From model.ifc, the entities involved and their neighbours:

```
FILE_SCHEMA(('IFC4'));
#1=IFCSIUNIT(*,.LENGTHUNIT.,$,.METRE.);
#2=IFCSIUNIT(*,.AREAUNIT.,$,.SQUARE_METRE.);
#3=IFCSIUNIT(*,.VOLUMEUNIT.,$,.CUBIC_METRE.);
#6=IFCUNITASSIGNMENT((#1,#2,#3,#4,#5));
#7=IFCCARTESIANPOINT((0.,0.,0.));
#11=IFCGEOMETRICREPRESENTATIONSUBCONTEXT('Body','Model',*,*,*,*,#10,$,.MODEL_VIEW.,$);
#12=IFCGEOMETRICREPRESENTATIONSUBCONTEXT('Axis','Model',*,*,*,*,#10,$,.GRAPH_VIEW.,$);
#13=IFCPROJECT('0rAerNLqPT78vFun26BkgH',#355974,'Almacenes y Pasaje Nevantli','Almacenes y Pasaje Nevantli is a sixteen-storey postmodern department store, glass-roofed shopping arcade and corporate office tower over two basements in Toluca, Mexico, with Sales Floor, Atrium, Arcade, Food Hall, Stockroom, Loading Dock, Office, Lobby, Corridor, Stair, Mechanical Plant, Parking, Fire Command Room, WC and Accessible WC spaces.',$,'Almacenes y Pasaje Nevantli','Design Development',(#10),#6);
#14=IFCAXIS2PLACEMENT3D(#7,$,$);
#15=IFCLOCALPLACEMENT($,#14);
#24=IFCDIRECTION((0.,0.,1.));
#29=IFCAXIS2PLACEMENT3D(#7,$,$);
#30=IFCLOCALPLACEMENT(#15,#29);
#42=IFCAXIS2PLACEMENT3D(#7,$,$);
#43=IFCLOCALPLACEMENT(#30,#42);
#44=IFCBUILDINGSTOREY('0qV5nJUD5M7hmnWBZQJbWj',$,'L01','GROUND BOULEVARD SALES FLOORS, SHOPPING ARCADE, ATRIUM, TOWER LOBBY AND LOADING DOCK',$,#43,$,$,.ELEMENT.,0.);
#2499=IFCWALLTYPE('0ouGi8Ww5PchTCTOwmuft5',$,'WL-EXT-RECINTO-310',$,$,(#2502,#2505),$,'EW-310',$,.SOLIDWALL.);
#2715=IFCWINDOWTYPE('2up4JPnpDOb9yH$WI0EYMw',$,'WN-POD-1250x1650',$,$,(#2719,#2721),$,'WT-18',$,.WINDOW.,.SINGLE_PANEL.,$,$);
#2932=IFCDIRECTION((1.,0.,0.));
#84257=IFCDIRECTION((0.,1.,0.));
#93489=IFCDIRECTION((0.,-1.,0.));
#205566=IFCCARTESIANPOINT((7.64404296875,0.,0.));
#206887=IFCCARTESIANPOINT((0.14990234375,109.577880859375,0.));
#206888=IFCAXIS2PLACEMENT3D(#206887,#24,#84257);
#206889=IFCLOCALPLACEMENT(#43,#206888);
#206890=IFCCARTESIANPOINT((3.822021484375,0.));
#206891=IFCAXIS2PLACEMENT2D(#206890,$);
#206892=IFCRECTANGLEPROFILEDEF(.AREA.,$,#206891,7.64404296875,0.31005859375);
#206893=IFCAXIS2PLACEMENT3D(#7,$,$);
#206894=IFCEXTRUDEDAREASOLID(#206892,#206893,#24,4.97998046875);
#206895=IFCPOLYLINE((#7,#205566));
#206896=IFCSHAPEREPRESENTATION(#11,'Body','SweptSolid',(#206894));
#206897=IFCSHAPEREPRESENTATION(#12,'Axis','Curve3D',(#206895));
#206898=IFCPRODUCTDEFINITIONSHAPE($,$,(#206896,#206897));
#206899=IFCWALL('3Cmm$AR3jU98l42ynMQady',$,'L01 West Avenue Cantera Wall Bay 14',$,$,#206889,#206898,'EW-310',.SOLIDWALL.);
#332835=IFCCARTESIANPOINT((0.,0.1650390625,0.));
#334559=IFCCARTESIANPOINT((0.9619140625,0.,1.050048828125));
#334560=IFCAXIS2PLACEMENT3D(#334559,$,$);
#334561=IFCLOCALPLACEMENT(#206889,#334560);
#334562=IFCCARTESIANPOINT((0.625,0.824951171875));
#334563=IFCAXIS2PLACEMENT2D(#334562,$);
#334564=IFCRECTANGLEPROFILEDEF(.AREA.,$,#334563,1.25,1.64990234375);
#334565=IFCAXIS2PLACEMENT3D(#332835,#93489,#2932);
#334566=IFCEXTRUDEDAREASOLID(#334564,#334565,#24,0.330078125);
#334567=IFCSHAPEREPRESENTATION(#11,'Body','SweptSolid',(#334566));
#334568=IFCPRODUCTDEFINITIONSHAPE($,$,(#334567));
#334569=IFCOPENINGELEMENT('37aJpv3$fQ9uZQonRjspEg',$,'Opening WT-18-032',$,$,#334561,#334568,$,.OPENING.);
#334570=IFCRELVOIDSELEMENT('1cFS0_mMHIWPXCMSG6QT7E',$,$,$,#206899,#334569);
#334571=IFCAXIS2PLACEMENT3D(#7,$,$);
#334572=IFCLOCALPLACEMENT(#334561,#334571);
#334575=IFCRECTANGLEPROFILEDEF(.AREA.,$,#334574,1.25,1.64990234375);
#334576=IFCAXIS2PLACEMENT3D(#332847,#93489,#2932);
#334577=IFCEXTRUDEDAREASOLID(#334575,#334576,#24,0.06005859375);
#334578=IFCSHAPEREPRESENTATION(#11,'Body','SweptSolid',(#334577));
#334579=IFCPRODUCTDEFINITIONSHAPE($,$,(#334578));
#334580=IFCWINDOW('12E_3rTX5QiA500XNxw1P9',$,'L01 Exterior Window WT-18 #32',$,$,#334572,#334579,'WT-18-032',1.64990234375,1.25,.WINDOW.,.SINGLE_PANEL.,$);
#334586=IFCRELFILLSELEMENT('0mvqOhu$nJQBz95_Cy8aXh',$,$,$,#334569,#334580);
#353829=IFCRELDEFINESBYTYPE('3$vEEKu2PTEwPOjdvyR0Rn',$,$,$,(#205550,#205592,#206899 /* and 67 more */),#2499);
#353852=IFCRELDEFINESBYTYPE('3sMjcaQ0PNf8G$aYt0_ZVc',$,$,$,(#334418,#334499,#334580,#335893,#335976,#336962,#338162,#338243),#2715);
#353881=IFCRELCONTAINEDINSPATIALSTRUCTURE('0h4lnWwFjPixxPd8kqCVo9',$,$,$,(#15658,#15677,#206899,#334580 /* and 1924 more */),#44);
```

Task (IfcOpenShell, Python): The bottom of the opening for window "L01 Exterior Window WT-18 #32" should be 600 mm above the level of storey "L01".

```python
import numpy as np
import ifcopenshell
import ifcopenshell.api.geometry
import ifcopenshell.geom
import ifcopenshell.util.element
import ifcopenshell.util.placement
import ifcopenshell.util.shape
import ifcopenshell.util.unit

model = ifcopenshell.open("model.ifc")
unit_scale = ifcopenshell.util.unit.calculate_unit_scale(model)

window = model.by_guid("12E_3rTX5QiA500XNxw1P9")
opening = window.FillsVoids[0].RelatingOpeningElement
storey = ifcopenshell.util.element.get_container(window, ifc_class="IfcBuildingStorey")
level = ifcopenshell.util.placement.get_local_placement(storey.ObjectPlacement)[2, 3]

# The opening's origin need not be at the sill, so measure its lowest point.
shape = ifcopenshell.geom.create_shape(ifcopenshell.geom.settings(), opening)
bottom = ifcopenshell.util.shape.get_shape_bottom_elevation(shape, shape.geometry) / unit_scale
dz = level + 0.6 / unit_scale - bottom

shift = np.array([0.0, 0.0, dz])
# The window is placed relative to its opening, so it follows when the opening moves.
matrix = ifcopenshell.util.placement.get_local_placement(opening.ObjectPlacement)
matrix[:3, 3] += shift
ifcopenshell.api.geometry.edit_object_placement(
    model, product=opening, matrix=matrix, is_si=False, should_transform_children=True
)

print(f"moved by {dz * unit_scale:+.3f} m")

model.write("model_edited.ifc")
```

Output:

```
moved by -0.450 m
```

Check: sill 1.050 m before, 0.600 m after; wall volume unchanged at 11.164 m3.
